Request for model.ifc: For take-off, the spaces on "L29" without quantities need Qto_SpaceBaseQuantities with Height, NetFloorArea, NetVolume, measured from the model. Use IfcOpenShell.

First a look at what the model holds.

```python
import ifcopenshell
import ifcopenshell.util.element
import ifcopenshell.util.unit

model = ifcopenshell.open("model.ifc")
print(model.schema)
for unit_type in ("LENGTHUNIT", "AREAUNIT", "VOLUMEUNIT"):
    print(unit_type, ifcopenshell.util.unit.calculate_unit_scale(model, unit_type))
storey = next(s for s in model.by_type("IfcBuildingStorey") if s.Name == "L29")
spaces = [e for e in ifcopenshell.util.element.get_decomposition(storey) if e.is_a("IfcSpace")]
for e in sorted(spaces, key=lambda e: e.id()):
    print(e.id(), e.is_a(), e.Name, list(ifcopenshell.util.element.get_psets(e, qtos_only=True)), sep=" | ")
```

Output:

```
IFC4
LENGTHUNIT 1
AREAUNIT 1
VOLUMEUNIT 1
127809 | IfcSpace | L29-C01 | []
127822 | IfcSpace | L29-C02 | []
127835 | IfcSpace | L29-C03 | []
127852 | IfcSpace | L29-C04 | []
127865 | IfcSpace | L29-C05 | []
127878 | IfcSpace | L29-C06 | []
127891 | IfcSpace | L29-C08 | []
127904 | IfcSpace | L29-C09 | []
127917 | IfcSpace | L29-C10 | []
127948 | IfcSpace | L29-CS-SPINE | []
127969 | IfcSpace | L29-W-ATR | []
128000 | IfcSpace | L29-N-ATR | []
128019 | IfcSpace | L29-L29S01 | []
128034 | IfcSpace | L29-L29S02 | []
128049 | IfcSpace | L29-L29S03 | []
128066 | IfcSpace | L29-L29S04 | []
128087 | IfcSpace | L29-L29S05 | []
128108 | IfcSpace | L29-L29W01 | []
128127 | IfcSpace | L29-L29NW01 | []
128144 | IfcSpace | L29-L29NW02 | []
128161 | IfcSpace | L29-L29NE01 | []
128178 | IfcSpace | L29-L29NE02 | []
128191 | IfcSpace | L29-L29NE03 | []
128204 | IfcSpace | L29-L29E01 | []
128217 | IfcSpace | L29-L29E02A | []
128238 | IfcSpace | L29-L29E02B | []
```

```python
import ifcopenshell
import ifcopenshell.api.pset
import ifcopenshell.geom
import ifcopenshell.util.element
import ifcopenshell.util.shape
import ifcopenshell.util.unit

model = ifcopenshell.open("model.ifc")
unit_scale = ifcopenshell.util.unit.calculate_unit_scale(model)
area_scale = ifcopenshell.util.unit.calculate_unit_scale(model, "AREAUNIT")
volume_scale = ifcopenshell.util.unit.calculate_unit_scale(model, "VOLUMEUNIT")
settings = ifcopenshell.geom.settings()

storey = next(s for s in model.by_type("IfcBuildingStorey") if s.Name == "L29")
spaces = [e for e in ifcopenshell.util.element.get_decomposition(storey) if e.is_a("IfcSpace")]

for e in sorted(spaces, key=lambda e: e.id()):
    if ifcopenshell.util.element.get_psets(e, qtos_only=True, should_inherit=False):
        continue
    # Geometry comes back in metres, in the element's own axes.
    shape = ifcopenshell.geom.create_shape(settings, e)
    values = {
        "Height": ifcopenshell.util.shape.get_z(shape.geometry) / unit_scale,
        "NetFloorArea": ifcopenshell.util.shape.get_footprint_area(shape.geometry) / area_scale,
        "NetVolume": ifcopenshell.util.shape.get_volume(shape.geometry) / volume_scale,
    }
    qto = ifcopenshell.api.pset.add_qto(model, product=e, name="Qto_SpaceBaseQuantities")
    ifcopenshell.api.pset.edit_qto(model, qto=qto, properties=values)
    print(e.id(), {k: round(v, 3) for k, v in values.items()})

model.write("model_updated.ifc")
```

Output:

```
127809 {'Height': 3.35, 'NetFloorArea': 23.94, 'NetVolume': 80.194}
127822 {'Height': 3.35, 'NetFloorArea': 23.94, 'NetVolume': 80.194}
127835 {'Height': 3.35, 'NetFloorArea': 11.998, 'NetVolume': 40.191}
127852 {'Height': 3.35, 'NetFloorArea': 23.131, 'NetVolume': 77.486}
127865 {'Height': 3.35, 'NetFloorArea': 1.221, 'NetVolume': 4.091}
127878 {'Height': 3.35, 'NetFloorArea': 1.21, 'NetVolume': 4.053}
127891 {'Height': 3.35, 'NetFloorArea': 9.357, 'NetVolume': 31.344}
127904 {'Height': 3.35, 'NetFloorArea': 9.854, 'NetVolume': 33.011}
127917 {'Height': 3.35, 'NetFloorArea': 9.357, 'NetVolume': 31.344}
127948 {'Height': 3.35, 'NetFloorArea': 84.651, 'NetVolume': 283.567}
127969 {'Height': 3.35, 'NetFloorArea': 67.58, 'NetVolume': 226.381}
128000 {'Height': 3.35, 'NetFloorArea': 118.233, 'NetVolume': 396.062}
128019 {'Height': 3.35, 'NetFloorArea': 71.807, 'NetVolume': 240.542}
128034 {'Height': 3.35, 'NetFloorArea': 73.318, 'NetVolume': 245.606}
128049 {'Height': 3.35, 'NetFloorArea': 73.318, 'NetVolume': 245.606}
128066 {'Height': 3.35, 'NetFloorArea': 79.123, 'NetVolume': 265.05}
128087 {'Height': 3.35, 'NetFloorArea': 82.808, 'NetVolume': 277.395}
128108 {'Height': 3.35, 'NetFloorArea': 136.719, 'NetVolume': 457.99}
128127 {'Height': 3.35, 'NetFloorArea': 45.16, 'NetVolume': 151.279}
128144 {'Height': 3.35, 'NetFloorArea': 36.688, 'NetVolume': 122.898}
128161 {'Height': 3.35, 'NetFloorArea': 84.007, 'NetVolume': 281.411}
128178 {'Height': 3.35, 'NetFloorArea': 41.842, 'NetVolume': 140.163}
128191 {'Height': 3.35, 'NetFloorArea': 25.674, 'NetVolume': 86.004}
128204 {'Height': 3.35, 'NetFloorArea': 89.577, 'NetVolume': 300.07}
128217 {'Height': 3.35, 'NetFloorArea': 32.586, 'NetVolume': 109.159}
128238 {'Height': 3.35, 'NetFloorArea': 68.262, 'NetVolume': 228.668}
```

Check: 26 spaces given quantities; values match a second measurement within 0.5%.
